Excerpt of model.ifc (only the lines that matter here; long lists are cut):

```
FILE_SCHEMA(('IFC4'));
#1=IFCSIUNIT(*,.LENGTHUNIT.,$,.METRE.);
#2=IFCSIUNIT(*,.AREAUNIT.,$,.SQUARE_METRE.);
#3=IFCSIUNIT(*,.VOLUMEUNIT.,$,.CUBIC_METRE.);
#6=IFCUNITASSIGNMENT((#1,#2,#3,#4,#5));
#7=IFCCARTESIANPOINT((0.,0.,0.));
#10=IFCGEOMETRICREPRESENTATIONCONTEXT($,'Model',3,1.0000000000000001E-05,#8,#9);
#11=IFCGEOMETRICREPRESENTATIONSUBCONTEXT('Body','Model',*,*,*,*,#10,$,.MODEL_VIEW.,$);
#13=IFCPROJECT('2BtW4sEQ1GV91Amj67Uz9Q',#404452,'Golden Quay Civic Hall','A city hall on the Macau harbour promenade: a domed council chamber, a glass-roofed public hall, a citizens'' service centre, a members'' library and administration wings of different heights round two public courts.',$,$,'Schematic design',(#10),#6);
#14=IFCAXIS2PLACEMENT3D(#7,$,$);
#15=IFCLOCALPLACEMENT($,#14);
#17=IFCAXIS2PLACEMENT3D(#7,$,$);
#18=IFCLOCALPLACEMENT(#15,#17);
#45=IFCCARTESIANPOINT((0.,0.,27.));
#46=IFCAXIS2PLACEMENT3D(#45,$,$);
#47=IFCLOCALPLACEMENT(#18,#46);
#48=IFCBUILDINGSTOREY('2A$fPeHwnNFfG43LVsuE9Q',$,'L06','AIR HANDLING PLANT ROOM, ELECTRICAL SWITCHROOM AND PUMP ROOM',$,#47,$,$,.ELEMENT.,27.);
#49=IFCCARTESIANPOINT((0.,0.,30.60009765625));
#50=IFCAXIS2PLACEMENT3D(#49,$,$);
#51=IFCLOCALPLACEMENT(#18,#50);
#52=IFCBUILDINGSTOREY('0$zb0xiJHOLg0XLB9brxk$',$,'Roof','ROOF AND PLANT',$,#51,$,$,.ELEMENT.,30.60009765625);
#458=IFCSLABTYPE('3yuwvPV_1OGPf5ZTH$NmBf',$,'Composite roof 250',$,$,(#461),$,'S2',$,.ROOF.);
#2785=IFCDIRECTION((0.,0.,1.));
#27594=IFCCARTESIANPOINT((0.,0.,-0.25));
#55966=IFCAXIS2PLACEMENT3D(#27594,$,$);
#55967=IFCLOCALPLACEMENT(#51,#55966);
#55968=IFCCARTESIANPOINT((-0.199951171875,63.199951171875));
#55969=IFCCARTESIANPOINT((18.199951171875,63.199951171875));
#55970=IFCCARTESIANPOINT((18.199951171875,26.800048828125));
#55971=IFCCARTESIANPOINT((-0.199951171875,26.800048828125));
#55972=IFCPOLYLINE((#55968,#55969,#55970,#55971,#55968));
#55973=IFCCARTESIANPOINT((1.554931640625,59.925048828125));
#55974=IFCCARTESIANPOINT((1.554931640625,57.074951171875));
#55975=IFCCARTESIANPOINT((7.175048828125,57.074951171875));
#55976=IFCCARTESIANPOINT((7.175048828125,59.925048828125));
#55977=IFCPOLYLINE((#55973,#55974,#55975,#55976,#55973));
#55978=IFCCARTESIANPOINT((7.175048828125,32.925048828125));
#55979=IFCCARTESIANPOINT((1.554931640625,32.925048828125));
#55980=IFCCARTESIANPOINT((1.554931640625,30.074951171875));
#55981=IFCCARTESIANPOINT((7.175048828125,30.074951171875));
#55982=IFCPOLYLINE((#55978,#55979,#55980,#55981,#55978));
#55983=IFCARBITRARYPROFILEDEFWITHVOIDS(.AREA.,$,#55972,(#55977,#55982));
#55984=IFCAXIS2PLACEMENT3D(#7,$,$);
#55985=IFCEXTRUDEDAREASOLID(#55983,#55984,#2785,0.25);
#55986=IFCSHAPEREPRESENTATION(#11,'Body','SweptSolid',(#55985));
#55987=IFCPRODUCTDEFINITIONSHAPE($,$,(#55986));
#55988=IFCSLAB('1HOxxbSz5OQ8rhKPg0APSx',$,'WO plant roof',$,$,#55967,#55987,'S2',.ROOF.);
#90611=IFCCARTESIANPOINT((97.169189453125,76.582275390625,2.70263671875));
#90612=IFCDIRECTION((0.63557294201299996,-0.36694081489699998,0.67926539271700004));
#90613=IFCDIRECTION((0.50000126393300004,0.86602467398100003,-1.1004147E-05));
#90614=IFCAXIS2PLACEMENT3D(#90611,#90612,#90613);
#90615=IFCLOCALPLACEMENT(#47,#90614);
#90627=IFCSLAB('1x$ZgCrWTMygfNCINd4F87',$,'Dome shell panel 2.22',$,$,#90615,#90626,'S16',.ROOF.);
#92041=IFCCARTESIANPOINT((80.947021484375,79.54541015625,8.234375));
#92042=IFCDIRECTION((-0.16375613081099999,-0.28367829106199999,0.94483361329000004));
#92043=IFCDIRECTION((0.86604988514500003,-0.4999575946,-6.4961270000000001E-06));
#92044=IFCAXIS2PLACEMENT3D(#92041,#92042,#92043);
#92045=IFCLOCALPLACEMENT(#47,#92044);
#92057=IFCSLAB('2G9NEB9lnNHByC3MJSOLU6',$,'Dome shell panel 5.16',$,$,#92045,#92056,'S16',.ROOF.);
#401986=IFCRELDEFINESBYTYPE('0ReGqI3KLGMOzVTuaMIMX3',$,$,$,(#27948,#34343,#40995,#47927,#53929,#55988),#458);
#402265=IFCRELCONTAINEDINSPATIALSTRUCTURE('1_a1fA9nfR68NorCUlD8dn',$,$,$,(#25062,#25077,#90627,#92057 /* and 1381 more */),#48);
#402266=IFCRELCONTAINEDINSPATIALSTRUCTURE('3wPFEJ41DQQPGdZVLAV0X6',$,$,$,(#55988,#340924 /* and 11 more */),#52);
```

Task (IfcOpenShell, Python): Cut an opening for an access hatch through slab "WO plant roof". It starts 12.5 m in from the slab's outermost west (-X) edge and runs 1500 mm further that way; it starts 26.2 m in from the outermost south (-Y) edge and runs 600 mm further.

```python
import numpy as np
import ifcopenshell
import ifcopenshell.api.feature
import ifcopenshell.api.geometry
import ifcopenshell.api.root
import ifcopenshell.geom
import ifcopenshell.util.placement
import ifcopenshell.util.representation
import ifcopenshell.util.shape
import ifcopenshell.util.unit

model = ifcopenshell.open("model.ifc")
unit_scale = ifcopenshell.util.unit.calculate_unit_scale(model)
settings = ifcopenshell.geom.settings()


def volume(element):
    """Net volume in cubic metres, openings subtracted."""
    shape = ifcopenshell.geom.create_shape(settings, element)
    return ifcopenshell.util.shape.get_volume(shape.geometry)


slab = model.by_id(55988)
before = volume(slab)

# Extent in the slab's own axes, in metres. The edges named are its -X and -Y sides.
slab_shape = ifcopenshell.geom.create_shape(settings, slab)
vertices = ifcopenshell.util.shape.get_vertices(slab_shape.geometry)
x_min, y_min, bottom = vertices.min(axis=0)
top = vertices[:, 2].max()

opening = ifcopenshell.api.root.create_entity(model, ifc_class="IfcOpeningElement", name="Access hatch opening", predefined_type="OPENING")
context = ifcopenshell.util.representation.get_context(model, "Model", "Body", "MODEL_VIEW")
width, depth = 1.5, 0.6
outline = [(0.0, 0.0), (width, 0.0), (width, depth), (0.0, depth), (0.0, 0.0)]
# Overshoot both faces by 50 mm so the cut is clean.
shape = ifcopenshell.api.geometry.add_slab_representation(
    model, context=context, depth=top - bottom + 0.1, polyline=outline
)
ifcopenshell.api.geometry.assign_representation(model, product=opening, representation=shape)

matrix = ifcopenshell.util.placement.get_local_placement(slab.ObjectPlacement)
matrix[:, 3] = matrix @ np.append(np.array([x_min + 12.5, y_min + 26.2, bottom - 0.05]) / unit_scale, 1.0)
ifcopenshell.api.geometry.edit_object_placement(model, product=opening, matrix=matrix, is_si=False)
ifcopenshell.api.feature.add_feature(model, feature=opening, element=slab)

after = volume(slab)

print(f"slab volume {before:.3f} -> {after:.3f} m3")

model.write("model_updated.ifc")
```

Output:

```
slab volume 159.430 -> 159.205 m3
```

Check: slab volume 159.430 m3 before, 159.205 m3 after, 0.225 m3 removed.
